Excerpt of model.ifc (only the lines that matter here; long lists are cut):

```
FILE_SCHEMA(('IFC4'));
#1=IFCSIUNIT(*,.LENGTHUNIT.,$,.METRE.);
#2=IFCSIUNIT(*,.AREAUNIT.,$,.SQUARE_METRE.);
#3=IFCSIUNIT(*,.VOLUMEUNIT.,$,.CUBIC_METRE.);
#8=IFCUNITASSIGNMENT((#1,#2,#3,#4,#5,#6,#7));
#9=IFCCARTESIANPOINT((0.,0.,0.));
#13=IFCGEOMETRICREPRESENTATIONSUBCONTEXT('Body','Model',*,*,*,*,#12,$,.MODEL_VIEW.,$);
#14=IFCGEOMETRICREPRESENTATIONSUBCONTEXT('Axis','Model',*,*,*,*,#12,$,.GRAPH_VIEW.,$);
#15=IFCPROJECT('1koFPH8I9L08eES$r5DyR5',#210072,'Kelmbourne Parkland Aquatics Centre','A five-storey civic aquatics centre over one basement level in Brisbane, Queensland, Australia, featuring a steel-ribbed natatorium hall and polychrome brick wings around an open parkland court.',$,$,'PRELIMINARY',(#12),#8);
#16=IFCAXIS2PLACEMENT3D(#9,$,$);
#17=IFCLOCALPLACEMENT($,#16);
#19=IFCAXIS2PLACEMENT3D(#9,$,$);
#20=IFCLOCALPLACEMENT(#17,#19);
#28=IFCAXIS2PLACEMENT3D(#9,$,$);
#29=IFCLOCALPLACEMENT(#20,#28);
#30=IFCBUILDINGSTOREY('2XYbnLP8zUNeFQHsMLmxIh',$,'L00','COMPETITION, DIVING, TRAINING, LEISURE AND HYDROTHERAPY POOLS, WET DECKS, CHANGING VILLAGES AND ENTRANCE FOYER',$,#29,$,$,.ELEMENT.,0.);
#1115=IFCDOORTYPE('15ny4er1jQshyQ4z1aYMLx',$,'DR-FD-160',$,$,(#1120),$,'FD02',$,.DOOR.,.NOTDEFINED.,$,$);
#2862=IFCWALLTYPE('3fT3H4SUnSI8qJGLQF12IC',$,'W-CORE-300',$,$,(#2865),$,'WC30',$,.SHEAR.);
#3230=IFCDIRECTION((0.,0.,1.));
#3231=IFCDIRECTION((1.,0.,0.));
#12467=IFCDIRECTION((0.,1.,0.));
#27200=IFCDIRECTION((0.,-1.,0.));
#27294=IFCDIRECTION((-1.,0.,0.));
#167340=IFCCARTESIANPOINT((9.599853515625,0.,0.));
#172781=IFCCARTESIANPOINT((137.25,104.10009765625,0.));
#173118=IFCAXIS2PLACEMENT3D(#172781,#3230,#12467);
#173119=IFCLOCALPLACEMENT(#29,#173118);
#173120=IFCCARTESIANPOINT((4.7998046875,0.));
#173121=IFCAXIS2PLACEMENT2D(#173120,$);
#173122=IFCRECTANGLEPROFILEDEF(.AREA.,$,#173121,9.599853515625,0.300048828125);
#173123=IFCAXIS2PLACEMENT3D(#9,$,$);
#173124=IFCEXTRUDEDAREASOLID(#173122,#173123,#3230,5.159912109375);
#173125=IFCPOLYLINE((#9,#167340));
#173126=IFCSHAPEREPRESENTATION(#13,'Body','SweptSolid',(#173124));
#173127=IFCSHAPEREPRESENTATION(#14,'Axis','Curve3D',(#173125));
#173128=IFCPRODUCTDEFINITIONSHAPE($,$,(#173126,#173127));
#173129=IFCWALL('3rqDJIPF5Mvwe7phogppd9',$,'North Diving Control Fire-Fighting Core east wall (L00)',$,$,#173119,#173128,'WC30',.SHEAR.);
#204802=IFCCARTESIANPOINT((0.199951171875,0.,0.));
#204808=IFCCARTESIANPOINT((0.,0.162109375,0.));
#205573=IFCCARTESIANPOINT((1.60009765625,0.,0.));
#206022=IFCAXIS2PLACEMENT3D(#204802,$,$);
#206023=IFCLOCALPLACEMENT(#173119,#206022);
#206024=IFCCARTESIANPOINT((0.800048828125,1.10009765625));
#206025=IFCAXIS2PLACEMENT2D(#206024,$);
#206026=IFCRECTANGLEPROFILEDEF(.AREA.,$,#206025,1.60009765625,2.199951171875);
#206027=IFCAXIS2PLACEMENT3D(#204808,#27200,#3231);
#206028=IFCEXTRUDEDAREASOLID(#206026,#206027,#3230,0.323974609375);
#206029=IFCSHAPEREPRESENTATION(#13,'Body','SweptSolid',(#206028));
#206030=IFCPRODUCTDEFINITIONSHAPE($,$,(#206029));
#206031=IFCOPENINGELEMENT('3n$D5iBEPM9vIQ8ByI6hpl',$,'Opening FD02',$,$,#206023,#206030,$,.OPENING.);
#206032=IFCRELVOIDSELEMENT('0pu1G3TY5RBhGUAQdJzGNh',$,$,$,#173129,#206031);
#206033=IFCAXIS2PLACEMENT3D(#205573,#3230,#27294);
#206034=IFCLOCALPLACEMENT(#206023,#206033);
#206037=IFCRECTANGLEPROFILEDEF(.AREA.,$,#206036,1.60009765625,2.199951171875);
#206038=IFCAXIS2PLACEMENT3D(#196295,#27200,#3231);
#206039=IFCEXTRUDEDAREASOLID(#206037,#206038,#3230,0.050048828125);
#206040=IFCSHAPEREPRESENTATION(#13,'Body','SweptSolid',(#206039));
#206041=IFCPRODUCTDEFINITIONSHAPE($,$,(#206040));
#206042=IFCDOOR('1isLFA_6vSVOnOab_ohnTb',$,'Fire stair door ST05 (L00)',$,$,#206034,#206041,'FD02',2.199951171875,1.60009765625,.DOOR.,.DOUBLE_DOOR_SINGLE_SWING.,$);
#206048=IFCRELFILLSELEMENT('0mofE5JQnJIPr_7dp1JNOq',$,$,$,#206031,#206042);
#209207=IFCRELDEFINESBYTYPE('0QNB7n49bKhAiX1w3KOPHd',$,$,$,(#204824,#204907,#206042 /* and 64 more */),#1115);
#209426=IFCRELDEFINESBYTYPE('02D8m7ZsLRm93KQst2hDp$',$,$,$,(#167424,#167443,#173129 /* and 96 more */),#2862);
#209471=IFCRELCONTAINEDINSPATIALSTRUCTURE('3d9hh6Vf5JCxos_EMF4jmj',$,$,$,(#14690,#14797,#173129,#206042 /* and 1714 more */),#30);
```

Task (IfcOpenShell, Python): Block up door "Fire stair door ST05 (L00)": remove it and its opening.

```python
import ifcopenshell
import ifcopenshell.api.feature
import ifcopenshell.api.root
import ifcopenshell.geom
import ifcopenshell.util.shape

model = ifcopenshell.open("model.ifc")
settings = ifcopenshell.geom.settings()


def volume(element):
    """Net volume in cubic metres, openings subtracted."""
    shape = ifcopenshell.geom.create_shape(settings, element)
    return ifcopenshell.util.shape.get_volume(shape.geometry)


door = model.by_id(206042)
opening = door.FillsVoids[0].RelatingOpeningElement
wall = opening.VoidsElements[0].RelatingBuildingElement
before = volume(wall)

ifcopenshell.api.root.remove_product(model, product=door)
ifcopenshell.api.feature.remove_feature(model, feature=opening)

after = volume(wall)

print(f"wall volume {before:.3f} -> {after:.3f} m3")

model.write("model_edited.ifc")
```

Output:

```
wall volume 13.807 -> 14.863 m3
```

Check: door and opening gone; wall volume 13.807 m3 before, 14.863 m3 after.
